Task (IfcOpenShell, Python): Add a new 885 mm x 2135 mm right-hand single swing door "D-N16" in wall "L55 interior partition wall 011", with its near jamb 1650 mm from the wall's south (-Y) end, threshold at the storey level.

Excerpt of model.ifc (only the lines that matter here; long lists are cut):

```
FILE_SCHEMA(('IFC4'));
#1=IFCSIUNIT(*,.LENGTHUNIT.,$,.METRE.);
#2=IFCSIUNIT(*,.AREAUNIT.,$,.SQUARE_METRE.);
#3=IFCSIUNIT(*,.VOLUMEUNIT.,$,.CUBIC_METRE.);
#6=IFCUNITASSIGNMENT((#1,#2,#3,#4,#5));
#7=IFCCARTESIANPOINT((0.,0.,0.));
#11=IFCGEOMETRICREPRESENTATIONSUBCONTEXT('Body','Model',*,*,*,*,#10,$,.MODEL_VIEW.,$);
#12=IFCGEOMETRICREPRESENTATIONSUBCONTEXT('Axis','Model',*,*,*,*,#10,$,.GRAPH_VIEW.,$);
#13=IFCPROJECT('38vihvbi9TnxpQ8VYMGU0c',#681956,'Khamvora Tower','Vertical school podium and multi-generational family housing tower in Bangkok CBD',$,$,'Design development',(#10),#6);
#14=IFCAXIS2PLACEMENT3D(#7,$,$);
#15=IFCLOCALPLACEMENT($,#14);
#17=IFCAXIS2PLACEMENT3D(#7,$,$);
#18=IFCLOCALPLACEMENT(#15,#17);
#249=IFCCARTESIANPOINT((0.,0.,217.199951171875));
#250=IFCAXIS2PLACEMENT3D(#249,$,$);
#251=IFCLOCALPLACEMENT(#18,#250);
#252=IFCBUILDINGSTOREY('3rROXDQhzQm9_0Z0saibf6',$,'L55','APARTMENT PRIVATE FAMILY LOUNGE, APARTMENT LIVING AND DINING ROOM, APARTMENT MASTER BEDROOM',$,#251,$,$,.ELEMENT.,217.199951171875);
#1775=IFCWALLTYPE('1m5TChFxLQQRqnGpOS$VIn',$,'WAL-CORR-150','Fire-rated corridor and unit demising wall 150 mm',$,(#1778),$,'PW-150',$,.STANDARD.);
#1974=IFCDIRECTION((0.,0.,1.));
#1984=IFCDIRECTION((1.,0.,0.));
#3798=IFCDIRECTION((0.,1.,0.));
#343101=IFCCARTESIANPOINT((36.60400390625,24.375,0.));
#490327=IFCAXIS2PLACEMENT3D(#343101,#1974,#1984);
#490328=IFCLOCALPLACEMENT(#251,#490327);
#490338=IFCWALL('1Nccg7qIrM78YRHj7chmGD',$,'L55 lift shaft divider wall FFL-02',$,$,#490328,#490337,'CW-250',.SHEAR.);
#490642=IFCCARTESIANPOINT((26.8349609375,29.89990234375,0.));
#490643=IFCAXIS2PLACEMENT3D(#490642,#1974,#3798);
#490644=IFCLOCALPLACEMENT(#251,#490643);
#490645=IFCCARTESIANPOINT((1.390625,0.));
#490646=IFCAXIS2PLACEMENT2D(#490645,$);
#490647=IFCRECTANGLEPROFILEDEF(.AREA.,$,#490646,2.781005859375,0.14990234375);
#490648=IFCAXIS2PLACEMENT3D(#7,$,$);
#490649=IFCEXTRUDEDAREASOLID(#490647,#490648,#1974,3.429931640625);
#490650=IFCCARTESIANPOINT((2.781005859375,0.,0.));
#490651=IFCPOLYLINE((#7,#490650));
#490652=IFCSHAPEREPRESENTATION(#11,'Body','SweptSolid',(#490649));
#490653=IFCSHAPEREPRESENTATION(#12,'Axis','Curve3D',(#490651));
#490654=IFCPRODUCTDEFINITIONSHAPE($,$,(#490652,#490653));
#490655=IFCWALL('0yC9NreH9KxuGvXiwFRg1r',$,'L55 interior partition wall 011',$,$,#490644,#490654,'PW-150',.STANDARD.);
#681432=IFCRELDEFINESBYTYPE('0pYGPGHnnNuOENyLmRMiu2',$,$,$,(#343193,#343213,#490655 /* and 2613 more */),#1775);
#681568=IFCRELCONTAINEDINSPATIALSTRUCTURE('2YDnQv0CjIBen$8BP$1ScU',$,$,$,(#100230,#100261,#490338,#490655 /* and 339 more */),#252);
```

```python
import numpy as np
import ifcopenshell
import ifcopenshell.api.feature
import ifcopenshell.api.geometry
import ifcopenshell.api.root
import ifcopenshell.api.spatial
import ifcopenshell.geom
import ifcopenshell.util.element
import ifcopenshell.util.placement
import ifcopenshell.util.representation
import ifcopenshell.util.shape
import ifcopenshell.util.unit

model = ifcopenshell.open("model.ifc")
unit_scale = ifcopenshell.util.unit.calculate_unit_scale(model)
settings = ifcopenshell.geom.settings()


def volume(element):
    """Net volume in cubic metres, openings subtracted."""
    shape = ifcopenshell.geom.create_shape(settings, element)
    return ifcopenshell.util.shape.get_volume(shape.geometry)


wall = model.by_guid("0yC9NreH9KxuGvXiwFRg1r")
storey = ifcopenshell.util.element.get_container(wall, ifc_class="IfcBuildingStorey")
context = ifcopenshell.util.representation.get_context(model, "Model", "Body", "MODEL_VIEW")
before = volume(wall)

width, height, from_end, sill = 0.885, 2.135, 1.65, 0.0  # metres

# The wall runs along its own X axis, and the end named is its -X end.
wall_shape = ifcopenshell.geom.create_shape(settings, wall)
x, y, z = ifcopenshell.util.shape.get_vertices(wall_shape.geometry).T
start = x.min() + from_end
face, thickness = float(y.min()), float(y.max() - y.min())
wall_matrix = ifcopenshell.util.placement.get_local_placement(wall.ObjectPlacement)
level = ifcopenshell.util.placement.get_local_placement(storey.ObjectPlacement)[2, 3]


def in_wall(x, y):
    """Placement at x, y metres in the wall's axes, at sill height."""
    matrix = wall_matrix.copy()
    matrix[:, 3] = wall_matrix @ np.array([x / unit_scale, y / unit_scale, 0.0, 1.0])
    matrix[2, 3] = level + sill / unit_scale
    return matrix


# Opening: a box that overshoots both wall faces by 50 mm.
opening = ifcopenshell.api.root.create_entity(model, ifc_class="IfcOpeningElement", predefined_type="OPENING")
box = ifcopenshell.api.geometry.add_wall_representation(
    model, context=context, length=width, height=height, thickness=thickness + 0.1
)
ifcopenshell.api.geometry.assign_representation(model, product=opening, representation=box)
ifcopenshell.api.geometry.edit_object_placement(model, product=opening, matrix=in_wall(start, face - 0.05), is_si=False)
ifcopenshell.api.feature.add_feature(model, feature=opening, element=wall)

door = ifcopenshell.api.root.create_entity(model, ifc_class="IfcDoor", name="D-N16", predefined_type="DOOR")
door.OverallWidth, door.OverallHeight = width / unit_scale, height / unit_scale
door.OperationType = "SINGLE_SWING_RIGHT"
body = ifcopenshell.api.geometry.add_door_representation(
    model,
    context=context,
    overall_width=door.OverallWidth,
    overall_height=door.OverallHeight,
    operation_type="SINGLE_SWING_RIGHT",
    lining_properties={"LiningDepth": thickness / unit_scale, "ThresholdDepth": thickness / unit_scale},
)
ifcopenshell.api.geometry.assign_representation(model, product=door, representation=body)
ifcopenshell.api.spatial.assign_container(model, products=[door], relating_structure=storey)
ifcopenshell.api.feature.add_filling(model, opening=opening, element=door)

# The lining spans the wall, so the door starts at the wall face.
ifcopenshell.api.geometry.edit_object_placement(model, product=door, matrix=in_wall(start, face), is_si=False)

after = volume(wall)

print(f"wall volume {before:.3f} -> {after:.3f} m3")

model.write("model_v2.ifc")
```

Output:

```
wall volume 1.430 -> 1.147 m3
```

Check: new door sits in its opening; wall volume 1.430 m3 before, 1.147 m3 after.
